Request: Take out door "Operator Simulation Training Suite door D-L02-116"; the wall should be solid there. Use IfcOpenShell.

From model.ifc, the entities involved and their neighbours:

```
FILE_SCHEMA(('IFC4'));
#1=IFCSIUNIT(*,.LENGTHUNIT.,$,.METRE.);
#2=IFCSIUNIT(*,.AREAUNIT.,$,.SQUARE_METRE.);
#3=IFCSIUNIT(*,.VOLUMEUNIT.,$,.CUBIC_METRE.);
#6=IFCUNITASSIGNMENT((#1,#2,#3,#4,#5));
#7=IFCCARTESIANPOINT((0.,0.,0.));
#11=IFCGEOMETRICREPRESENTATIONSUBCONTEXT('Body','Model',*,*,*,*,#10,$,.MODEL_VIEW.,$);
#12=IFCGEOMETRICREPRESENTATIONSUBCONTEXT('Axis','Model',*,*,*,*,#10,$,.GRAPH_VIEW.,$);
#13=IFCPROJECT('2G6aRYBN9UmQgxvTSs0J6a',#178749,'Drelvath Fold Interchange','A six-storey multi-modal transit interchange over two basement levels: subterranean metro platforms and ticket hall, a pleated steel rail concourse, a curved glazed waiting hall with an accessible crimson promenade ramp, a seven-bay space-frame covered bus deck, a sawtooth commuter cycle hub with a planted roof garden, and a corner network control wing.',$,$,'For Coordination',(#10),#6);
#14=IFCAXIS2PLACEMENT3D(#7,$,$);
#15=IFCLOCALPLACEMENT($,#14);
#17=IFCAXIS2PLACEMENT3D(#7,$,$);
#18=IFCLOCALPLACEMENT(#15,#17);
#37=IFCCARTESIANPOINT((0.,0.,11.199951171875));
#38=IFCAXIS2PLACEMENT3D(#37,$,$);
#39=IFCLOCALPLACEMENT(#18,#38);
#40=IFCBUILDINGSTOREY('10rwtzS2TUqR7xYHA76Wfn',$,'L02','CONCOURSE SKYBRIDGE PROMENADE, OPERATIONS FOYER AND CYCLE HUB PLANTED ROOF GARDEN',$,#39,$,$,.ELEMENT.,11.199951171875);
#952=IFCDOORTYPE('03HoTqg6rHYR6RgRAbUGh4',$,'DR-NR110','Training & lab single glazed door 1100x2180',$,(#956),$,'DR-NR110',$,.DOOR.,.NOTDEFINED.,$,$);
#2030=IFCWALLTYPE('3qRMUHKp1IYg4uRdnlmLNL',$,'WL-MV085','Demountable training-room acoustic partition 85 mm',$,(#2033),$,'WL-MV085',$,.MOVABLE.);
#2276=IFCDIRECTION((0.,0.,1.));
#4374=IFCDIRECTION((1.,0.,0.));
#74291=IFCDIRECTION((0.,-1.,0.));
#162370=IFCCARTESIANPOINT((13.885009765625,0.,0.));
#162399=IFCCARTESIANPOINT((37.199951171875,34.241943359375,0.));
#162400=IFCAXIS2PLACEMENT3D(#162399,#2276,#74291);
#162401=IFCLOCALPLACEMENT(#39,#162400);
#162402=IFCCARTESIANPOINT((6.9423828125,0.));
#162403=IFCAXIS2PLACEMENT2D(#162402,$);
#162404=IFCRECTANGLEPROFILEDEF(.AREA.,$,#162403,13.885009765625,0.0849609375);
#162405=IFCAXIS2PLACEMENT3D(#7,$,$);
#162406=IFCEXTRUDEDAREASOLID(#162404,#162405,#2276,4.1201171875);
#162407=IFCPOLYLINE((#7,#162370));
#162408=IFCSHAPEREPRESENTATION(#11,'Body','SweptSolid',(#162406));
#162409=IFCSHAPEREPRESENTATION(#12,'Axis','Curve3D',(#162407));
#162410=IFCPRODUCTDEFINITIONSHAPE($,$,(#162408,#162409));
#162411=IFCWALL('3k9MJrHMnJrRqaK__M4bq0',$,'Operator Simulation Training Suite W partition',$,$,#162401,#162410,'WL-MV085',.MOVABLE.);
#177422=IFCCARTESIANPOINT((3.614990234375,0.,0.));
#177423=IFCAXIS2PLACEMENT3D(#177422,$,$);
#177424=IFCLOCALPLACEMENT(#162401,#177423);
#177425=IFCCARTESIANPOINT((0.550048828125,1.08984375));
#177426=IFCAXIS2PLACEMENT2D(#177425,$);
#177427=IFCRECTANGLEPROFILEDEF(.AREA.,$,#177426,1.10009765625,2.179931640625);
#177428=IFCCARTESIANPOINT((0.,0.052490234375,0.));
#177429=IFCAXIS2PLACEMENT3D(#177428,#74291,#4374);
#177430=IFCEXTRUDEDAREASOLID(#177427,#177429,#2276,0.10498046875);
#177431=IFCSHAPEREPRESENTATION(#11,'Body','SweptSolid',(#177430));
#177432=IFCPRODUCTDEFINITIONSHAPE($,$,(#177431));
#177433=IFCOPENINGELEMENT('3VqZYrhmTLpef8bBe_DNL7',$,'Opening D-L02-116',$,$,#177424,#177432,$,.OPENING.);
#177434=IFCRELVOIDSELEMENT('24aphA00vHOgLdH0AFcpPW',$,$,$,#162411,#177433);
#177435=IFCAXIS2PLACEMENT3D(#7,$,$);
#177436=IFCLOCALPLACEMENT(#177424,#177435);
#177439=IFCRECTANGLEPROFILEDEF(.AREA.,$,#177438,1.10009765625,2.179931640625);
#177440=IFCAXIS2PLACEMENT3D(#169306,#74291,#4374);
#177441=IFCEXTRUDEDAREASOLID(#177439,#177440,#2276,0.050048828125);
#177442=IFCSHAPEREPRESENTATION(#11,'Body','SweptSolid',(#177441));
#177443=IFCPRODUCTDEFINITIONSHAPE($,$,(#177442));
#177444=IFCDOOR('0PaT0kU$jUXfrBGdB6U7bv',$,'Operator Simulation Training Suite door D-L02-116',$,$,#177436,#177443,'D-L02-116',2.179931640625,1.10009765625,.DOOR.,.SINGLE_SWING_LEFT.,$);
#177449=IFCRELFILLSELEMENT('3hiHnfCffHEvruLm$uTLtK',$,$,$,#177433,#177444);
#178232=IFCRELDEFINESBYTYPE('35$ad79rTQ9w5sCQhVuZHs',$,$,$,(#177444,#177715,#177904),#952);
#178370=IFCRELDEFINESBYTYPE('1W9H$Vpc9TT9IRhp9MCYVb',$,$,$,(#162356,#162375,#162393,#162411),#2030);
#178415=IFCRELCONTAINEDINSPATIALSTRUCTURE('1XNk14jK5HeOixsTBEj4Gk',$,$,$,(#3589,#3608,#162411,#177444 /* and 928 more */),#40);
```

```python
import ifcopenshell
import ifcopenshell.api.feature
import ifcopenshell.api.root
import ifcopenshell.geom
import ifcopenshell.util.shape

model = ifcopenshell.open("model.ifc")
settings = ifcopenshell.geom.settings()


def volume(element):
    """Net volume in cubic metres, openings subtracted."""
    shape = ifcopenshell.geom.create_shape(settings, element)
    return ifcopenshell.util.shape.get_volume(shape.geometry)


door = model.by_guid("0PaT0kU$jUXfrBGdB6U7bv")
opening = door.FillsVoids[0].RelatingOpeningElement
wall = opening.VoidsElements[0].RelatingBuildingElement
before = volume(wall)

ifcopenshell.api.root.remove_product(model, product=door)
ifcopenshell.api.feature.remove_feature(model, feature=opening)

after = volume(wall)

print(f"wall volume {before:.3f} -> {after:.3f} m3")

model.write("model_v2.ifc")
```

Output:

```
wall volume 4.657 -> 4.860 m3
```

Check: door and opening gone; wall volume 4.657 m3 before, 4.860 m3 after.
